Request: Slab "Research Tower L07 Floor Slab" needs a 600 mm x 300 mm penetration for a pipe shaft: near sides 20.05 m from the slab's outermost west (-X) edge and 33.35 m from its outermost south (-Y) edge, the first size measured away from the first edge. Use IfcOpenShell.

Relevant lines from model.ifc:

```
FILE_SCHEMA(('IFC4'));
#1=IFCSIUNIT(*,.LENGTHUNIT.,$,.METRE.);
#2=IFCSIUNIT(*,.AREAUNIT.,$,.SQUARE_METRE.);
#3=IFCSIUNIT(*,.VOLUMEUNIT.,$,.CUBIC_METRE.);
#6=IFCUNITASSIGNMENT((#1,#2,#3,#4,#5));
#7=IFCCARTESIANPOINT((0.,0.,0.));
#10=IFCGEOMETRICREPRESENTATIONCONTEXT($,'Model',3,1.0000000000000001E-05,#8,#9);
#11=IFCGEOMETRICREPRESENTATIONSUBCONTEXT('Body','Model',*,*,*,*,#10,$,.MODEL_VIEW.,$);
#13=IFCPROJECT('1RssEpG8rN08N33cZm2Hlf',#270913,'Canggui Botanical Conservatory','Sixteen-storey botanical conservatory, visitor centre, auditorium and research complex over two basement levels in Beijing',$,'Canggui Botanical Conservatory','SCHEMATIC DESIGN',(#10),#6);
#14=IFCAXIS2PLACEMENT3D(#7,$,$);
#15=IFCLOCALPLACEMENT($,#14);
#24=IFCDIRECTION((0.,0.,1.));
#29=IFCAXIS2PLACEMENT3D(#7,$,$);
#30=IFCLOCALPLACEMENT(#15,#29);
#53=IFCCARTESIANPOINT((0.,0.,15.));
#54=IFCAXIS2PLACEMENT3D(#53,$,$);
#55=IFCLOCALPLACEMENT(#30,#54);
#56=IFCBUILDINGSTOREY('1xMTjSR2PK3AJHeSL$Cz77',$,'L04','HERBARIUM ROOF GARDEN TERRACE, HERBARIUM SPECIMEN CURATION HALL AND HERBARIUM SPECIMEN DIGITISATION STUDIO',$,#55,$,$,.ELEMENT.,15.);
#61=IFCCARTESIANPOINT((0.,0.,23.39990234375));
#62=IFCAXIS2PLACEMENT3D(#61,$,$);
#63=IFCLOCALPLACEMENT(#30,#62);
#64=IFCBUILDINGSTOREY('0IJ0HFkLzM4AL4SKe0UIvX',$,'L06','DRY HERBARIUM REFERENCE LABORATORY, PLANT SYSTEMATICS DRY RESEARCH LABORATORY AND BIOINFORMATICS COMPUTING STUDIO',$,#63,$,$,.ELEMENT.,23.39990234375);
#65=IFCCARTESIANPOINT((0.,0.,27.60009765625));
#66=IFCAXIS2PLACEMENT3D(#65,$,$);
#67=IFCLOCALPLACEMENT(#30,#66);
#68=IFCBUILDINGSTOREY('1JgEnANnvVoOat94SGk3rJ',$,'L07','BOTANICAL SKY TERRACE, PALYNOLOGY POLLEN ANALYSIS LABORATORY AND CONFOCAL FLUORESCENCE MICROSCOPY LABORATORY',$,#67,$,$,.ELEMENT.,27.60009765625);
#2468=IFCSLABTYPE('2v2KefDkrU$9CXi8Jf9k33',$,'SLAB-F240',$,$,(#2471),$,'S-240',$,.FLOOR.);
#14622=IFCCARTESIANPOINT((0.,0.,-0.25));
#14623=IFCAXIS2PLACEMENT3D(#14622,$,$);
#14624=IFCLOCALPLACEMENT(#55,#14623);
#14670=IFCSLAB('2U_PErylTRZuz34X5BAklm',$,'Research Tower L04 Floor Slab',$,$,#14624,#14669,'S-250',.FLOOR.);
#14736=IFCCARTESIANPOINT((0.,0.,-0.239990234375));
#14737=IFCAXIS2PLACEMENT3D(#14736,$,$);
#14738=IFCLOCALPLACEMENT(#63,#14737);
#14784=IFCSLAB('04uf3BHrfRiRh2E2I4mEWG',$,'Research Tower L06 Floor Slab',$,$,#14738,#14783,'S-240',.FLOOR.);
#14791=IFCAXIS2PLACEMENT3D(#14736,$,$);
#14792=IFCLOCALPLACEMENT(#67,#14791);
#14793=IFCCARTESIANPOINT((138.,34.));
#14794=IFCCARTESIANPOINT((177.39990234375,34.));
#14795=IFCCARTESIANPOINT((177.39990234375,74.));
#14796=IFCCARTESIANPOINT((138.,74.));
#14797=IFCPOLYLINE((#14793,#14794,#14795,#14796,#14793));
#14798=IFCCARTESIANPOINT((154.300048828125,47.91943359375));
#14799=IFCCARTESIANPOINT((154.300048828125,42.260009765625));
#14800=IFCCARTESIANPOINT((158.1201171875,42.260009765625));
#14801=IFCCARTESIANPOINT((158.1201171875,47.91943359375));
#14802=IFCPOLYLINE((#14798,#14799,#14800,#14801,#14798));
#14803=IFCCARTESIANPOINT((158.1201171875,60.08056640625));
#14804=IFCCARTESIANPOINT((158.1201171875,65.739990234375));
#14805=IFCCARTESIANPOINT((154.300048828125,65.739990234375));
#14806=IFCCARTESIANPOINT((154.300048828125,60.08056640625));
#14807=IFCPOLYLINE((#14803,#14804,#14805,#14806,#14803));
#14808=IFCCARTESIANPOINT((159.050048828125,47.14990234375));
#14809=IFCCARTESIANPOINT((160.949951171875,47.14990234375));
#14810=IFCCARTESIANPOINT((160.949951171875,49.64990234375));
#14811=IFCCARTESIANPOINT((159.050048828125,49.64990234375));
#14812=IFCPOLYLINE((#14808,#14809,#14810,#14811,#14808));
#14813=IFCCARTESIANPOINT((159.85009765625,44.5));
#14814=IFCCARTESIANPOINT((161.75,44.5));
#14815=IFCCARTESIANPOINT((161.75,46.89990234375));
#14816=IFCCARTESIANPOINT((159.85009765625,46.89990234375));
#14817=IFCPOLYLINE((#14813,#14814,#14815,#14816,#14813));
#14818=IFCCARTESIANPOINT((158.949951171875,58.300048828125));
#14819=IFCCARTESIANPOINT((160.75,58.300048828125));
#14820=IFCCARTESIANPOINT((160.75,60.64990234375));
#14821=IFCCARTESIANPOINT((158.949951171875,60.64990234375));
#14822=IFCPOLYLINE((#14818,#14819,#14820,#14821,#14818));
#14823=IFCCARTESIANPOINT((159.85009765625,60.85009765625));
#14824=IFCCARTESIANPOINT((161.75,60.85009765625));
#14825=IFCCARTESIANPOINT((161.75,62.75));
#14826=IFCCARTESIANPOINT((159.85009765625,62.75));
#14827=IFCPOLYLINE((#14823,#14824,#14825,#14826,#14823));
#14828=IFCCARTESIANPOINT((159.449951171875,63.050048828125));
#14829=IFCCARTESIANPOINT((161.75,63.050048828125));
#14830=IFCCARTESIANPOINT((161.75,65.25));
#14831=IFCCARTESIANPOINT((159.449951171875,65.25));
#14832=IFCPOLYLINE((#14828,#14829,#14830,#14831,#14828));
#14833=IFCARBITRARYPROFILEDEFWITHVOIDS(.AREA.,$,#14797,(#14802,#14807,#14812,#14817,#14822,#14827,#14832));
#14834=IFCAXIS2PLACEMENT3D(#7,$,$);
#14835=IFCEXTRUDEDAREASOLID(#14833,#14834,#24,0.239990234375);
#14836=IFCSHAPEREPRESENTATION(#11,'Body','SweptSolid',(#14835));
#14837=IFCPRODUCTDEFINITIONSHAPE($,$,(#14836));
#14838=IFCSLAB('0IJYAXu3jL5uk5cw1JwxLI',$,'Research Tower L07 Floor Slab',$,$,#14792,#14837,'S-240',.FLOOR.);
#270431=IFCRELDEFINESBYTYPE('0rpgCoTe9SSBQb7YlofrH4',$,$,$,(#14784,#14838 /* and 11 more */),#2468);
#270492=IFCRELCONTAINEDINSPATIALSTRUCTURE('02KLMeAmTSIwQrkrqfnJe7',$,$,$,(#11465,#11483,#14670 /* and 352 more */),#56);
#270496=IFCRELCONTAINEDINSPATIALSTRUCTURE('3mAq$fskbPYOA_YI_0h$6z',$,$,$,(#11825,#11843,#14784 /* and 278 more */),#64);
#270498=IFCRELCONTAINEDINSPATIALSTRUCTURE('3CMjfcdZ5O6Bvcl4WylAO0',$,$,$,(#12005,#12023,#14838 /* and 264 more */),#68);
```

```python
import numpy as np
import ifcopenshell
import ifcopenshell.api.feature
import ifcopenshell.api.geometry
import ifcopenshell.api.root
import ifcopenshell.geom
import ifcopenshell.util.placement
import ifcopenshell.util.representation
import ifcopenshell.util.shape
import ifcopenshell.util.unit

model = ifcopenshell.open("model.ifc")
unit_scale = ifcopenshell.util.unit.calculate_unit_scale(model)
settings = ifcopenshell.geom.settings()


def volume(element):
    """Net volume in cubic metres, openings subtracted."""
    shape = ifcopenshell.geom.create_shape(settings, element)
    return ifcopenshell.util.shape.get_volume(shape.geometry)


slab = model.by_guid("0IJYAXu3jL5uk5cw1JwxLI")
before = volume(slab)

# Extent in the slab's own axes, in metres. The edges named are its -X and -Y sides.
slab_shape = ifcopenshell.geom.create_shape(settings, slab)
vertices = ifcopenshell.util.shape.get_vertices(slab_shape.geometry)
x_min, y_min, bottom = vertices.min(axis=0)
top = vertices[:, 2].max()

opening = ifcopenshell.api.root.create_entity(model, ifc_class="IfcOpeningElement", name="Pipe shaft opening", predefined_type="OPENING")
context = ifcopenshell.util.representation.get_context(model, "Model", "Body", "MODEL_VIEW")
width, depth = 0.6, 0.3
outline = [(0.0, 0.0), (width, 0.0), (width, depth), (0.0, depth), (0.0, 0.0)]
# Overshoot both faces by 50 mm so the cut is clean.
shape = ifcopenshell.api.geometry.add_slab_representation(
    model, context=context, depth=top - bottom + 0.1, polyline=outline
)
ifcopenshell.api.geometry.assign_representation(model, product=opening, representation=shape)

matrix = ifcopenshell.util.placement.get_local_placement(slab.ObjectPlacement)
matrix[:, 3] = matrix @ np.append(np.array([x_min + 20.05, y_min + 33.35, bottom - 0.05]) / unit_scale, 1.0)
ifcopenshell.api.geometry.edit_object_placement(model, product=opening, matrix=matrix, is_si=False)
ifcopenshell.api.feature.add_feature(model, feature=opening, element=slab)

after = volume(slab)

print(f"slab volume {before:.3f} -> {after:.3f} m3")

model.write("model_v2.ifc")
```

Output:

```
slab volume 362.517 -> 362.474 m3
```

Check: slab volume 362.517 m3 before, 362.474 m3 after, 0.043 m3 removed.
